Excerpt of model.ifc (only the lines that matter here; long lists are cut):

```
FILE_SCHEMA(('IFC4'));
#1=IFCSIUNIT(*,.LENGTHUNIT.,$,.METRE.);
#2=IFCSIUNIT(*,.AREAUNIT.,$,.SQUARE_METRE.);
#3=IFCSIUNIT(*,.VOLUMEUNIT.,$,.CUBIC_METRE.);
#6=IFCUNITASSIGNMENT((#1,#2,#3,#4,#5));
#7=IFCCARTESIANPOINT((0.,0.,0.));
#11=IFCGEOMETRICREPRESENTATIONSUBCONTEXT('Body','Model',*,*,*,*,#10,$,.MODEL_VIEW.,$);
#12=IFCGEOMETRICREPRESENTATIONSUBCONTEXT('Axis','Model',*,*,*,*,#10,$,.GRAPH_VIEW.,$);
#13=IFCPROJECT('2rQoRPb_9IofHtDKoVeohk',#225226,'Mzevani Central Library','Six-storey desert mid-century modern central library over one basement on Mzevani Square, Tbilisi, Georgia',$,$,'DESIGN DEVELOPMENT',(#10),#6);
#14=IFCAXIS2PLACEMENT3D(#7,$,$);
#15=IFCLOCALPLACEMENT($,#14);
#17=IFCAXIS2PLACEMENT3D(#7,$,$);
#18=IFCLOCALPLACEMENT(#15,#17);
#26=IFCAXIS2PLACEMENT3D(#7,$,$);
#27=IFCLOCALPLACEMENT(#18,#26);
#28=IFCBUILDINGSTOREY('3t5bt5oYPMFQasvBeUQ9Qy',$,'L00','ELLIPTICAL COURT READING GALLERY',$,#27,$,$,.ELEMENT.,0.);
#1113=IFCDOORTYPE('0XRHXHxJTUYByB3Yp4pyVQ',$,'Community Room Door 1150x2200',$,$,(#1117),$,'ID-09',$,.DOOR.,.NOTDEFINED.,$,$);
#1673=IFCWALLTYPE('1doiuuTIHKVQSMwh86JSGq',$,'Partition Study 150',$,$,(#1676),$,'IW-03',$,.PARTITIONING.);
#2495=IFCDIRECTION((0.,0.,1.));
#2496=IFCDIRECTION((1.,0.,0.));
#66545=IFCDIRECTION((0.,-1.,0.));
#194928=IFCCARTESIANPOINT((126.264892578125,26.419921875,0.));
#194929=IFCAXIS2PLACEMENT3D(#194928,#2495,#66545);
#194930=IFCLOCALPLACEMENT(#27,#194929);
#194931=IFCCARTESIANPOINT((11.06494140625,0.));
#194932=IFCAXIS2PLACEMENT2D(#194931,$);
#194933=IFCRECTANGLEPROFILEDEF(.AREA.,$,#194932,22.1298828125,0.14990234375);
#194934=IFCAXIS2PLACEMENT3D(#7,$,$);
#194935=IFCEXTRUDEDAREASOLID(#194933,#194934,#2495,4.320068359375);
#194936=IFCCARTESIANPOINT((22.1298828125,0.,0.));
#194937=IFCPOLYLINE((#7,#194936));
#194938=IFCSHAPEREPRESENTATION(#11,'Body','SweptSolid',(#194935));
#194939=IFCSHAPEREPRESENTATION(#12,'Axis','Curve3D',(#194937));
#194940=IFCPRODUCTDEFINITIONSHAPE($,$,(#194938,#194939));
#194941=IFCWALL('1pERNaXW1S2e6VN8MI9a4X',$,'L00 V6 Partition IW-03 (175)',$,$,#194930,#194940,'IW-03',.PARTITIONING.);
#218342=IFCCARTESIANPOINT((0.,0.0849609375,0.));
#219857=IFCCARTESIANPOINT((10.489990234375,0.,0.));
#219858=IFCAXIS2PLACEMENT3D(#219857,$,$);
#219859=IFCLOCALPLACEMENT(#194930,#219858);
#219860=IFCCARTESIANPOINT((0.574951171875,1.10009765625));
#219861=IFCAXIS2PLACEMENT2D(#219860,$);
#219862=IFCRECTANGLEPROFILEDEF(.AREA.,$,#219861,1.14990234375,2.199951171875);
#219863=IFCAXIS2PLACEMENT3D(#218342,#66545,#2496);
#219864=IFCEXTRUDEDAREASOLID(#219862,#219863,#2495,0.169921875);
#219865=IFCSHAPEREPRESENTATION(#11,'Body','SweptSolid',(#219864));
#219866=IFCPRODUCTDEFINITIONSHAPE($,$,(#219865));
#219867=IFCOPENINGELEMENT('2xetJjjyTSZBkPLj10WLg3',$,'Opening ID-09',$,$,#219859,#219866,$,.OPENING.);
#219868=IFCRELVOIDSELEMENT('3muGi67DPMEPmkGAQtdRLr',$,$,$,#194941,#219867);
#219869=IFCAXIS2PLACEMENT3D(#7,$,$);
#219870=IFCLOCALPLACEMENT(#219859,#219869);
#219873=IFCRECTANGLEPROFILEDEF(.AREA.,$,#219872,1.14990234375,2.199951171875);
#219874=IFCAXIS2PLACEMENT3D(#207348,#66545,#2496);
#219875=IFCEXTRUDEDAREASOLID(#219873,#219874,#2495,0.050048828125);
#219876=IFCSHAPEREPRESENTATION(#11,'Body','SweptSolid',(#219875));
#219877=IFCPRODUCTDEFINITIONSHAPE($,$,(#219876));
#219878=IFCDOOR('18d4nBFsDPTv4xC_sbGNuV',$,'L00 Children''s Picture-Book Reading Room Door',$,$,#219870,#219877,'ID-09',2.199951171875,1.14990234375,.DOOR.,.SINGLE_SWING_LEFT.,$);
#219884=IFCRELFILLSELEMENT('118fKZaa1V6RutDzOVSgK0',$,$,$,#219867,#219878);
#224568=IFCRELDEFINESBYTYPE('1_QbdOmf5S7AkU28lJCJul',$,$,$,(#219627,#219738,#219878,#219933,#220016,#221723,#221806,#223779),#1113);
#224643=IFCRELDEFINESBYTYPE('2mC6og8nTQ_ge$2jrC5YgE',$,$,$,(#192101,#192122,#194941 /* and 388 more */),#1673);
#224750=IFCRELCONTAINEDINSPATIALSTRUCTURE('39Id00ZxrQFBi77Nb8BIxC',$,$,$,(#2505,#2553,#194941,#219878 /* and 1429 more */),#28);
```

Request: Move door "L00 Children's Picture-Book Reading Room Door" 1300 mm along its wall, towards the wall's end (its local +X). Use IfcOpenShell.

```python
import ifcopenshell
import ifcopenshell.api.geometry
import ifcopenshell.util.placement
import ifcopenshell.util.unit

model = ifcopenshell.open("model.ifc")
unit_scale = ifcopenshell.util.unit.calculate_unit_scale(model)

door = model.by_guid("18d4nBFsDPTv4xC_sbGNuV")
opening = door.FillsVoids[0].RelatingOpeningElement
wall = opening.VoidsElements[0].RelatingBuildingElement

wall_matrix = ifcopenshell.util.placement.get_local_placement(wall.ObjectPlacement)
shift = wall_matrix[:3, 0] * 1.3 / unit_scale
before = ifcopenshell.util.placement.get_local_placement(door.ObjectPlacement)[:3, 3].copy()

# The door is placed relative to its opening, so it follows when the opening moves.
matrix = ifcopenshell.util.placement.get_local_placement(opening.ObjectPlacement)
matrix[:3, 3] += shift
ifcopenshell.api.geometry.edit_object_placement(
    model, product=opening, matrix=matrix, is_si=False, should_transform_children=True
)

after = ifcopenshell.util.placement.get_local_placement(door.ObjectPlacement)[:3, 3]
print("door moved by", (after - before).round(3) + 0.0)

model.write("model_updated.ifc")
```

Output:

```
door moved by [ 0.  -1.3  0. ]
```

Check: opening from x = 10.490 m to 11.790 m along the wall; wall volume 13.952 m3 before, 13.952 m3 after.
